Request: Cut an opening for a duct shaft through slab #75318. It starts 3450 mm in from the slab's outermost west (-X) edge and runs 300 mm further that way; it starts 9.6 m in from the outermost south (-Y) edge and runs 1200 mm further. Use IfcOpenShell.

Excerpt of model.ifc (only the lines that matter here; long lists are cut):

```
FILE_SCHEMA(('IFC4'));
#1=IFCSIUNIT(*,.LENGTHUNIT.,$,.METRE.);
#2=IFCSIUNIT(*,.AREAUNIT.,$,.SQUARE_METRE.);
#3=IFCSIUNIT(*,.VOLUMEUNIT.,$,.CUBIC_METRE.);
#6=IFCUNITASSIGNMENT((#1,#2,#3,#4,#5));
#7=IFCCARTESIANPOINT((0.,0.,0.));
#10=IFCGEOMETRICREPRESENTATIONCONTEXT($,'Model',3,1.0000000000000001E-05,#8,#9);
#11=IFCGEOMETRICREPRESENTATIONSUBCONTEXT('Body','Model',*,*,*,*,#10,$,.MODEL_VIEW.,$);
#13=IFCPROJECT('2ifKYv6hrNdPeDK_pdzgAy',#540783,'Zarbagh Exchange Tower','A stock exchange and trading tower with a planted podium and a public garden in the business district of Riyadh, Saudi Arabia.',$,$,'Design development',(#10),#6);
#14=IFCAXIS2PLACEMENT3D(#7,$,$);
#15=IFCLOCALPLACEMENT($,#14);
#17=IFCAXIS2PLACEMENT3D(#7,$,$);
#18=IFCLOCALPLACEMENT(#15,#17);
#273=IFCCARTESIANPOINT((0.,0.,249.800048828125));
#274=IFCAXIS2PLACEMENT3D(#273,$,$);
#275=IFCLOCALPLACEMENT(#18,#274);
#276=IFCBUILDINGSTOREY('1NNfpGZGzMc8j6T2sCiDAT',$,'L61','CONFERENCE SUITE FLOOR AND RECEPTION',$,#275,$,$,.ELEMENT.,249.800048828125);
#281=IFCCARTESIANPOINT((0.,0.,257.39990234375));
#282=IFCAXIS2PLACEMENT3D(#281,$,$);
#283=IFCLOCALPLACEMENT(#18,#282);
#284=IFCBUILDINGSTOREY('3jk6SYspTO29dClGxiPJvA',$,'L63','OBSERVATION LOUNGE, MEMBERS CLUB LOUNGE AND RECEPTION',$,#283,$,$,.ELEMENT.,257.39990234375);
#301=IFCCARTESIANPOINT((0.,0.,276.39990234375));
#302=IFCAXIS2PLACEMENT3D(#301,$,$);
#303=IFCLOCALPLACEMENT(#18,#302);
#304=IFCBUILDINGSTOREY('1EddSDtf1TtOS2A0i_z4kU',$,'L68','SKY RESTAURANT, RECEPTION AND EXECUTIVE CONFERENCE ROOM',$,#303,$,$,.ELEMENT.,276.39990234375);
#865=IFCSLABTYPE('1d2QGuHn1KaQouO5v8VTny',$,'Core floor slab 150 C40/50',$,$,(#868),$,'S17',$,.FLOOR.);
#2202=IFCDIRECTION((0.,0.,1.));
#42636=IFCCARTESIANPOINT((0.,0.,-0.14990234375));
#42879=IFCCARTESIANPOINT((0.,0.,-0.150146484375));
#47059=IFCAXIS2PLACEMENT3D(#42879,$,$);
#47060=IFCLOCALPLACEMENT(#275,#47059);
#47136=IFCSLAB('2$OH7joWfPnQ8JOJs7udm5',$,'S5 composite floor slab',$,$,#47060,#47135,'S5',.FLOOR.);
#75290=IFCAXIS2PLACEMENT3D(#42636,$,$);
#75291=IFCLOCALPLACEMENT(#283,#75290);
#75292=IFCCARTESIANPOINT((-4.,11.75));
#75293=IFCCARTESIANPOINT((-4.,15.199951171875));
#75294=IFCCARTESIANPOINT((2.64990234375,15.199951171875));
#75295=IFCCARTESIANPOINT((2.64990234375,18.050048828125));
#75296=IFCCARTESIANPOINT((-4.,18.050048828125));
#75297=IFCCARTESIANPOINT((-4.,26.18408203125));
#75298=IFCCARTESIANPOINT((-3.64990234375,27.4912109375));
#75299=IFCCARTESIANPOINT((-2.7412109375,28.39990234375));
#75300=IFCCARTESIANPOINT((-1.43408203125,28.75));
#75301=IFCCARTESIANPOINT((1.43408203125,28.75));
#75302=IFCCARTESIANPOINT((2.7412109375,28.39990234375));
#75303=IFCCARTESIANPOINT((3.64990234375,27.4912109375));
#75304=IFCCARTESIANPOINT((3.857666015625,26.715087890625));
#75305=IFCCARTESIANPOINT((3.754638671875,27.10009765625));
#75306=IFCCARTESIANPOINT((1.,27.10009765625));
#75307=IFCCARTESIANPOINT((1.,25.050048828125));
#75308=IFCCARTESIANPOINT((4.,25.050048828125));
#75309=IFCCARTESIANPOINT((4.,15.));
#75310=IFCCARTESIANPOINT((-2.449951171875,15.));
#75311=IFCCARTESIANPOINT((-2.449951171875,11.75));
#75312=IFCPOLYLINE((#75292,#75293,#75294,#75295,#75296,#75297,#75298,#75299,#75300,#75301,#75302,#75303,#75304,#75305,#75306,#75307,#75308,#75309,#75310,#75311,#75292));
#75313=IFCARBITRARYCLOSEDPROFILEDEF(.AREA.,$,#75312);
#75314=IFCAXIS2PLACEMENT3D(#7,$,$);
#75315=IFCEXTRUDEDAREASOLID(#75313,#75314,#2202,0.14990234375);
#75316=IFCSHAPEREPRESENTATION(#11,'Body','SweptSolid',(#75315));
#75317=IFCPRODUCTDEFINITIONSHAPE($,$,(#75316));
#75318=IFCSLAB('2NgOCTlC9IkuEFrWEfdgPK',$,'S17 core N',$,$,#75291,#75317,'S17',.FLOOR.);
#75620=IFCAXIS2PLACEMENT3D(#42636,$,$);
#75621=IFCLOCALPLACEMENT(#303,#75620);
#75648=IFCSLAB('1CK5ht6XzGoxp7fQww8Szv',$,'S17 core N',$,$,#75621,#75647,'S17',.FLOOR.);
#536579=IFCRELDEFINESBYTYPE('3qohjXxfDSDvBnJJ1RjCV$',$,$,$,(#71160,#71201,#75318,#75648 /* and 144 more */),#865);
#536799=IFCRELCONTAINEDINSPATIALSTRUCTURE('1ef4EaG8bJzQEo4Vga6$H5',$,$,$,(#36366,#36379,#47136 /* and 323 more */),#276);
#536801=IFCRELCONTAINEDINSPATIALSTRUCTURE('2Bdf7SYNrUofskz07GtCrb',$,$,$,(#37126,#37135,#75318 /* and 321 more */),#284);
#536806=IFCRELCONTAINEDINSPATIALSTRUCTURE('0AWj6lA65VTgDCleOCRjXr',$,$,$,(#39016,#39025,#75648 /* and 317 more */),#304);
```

```python
import numpy as np
import ifcopenshell
import ifcopenshell.api.feature
import ifcopenshell.api.geometry
import ifcopenshell.api.root
import ifcopenshell.geom
import ifcopenshell.util.placement
import ifcopenshell.util.representation
import ifcopenshell.util.shape
import ifcopenshell.util.unit

model = ifcopenshell.open("model.ifc")
unit_scale = ifcopenshell.util.unit.calculate_unit_scale(model)
settings = ifcopenshell.geom.settings()


def volume(element):
    """Net volume in cubic metres, openings subtracted."""
    shape = ifcopenshell.geom.create_shape(settings, element)
    return ifcopenshell.util.shape.get_volume(shape.geometry)


slab = model.by_guid("2NgOCTlC9IkuEFrWEfdgPK")
before = volume(slab)

# Extent in the slab's own axes, in metres. The edges named are its -X and -Y sides.
slab_shape = ifcopenshell.geom.create_shape(settings, slab)
vertices = ifcopenshell.util.shape.get_vertices(slab_shape.geometry)
x_min, y_min, bottom = vertices.min(axis=0)
top = vertices[:, 2].max()

opening = ifcopenshell.api.root.create_entity(model, ifc_class="IfcOpeningElement", name="Duct shaft opening", predefined_type="OPENING")
context = ifcopenshell.util.representation.get_context(model, "Model", "Body", "MODEL_VIEW")
width, depth = 0.3, 1.2
outline = [(0.0, 0.0), (width, 0.0), (width, depth), (0.0, depth), (0.0, 0.0)]
# Overshoot both faces by 50 mm so the cut is clean.
shape = ifcopenshell.api.geometry.add_slab_representation(
    model, context=context, depth=top - bottom + 0.1, polyline=outline
)
ifcopenshell.api.geometry.assign_representation(model, product=opening, representation=shape)

matrix = ifcopenshell.util.placement.get_local_placement(slab.ObjectPlacement)
matrix[:, 3] = matrix @ np.append(np.array([x_min + 3.45, y_min + 9.6, bottom - 0.05]) / unit_scale, 1.0)
ifcopenshell.api.geometry.edit_object_placement(model, product=opening, matrix=matrix, is_si=False)
ifcopenshell.api.feature.add_feature(model, feature=opening, element=slab)

after = volume(slab)

print(f"slab volume {before:.3f} -> {after:.3f} m3")

model.write("model_v2.ifc")
```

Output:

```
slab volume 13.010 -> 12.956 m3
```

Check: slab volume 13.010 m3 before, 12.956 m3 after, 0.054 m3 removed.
